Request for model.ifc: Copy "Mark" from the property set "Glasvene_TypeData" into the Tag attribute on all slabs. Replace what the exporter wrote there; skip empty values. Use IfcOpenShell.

First a look at what the model holds.

```python
import ifcopenshell
import ifcopenshell.util.element

model = ifcopenshell.open("model.ifc")
print(model.schema)
slabs = model.by_type("IfcSlab")
print(len(slabs), "slabs")
for e in slabs[:8]:
    source = ifcopenshell.util.element.get_pset(e, "Glasvene_TypeData", "Mark")
    target = e.Tag
    print(e.id(), repr(source), repr(target), sep=" | ")
```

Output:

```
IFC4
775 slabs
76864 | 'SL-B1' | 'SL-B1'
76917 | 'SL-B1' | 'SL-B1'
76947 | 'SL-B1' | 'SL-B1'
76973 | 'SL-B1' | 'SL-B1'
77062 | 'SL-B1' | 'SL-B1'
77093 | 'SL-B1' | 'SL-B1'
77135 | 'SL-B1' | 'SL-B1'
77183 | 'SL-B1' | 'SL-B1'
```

```python
import ifcopenshell
import ifcopenshell.util.element

model = ifcopenshell.open("model.ifc")

count = 0
for e in model.by_type("IfcSlab"):
    value = ifcopenshell.util.element.get_pset(e, "Glasvene_TypeData", "Mark")
    current = e.Tag
    if not value or not value.strip() or current == value:
        continue
    e.Tag = value
    count += 1

print(count, "slabs updated")

model.write("model_v2.ifc")
```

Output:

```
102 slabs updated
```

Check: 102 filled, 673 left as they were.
